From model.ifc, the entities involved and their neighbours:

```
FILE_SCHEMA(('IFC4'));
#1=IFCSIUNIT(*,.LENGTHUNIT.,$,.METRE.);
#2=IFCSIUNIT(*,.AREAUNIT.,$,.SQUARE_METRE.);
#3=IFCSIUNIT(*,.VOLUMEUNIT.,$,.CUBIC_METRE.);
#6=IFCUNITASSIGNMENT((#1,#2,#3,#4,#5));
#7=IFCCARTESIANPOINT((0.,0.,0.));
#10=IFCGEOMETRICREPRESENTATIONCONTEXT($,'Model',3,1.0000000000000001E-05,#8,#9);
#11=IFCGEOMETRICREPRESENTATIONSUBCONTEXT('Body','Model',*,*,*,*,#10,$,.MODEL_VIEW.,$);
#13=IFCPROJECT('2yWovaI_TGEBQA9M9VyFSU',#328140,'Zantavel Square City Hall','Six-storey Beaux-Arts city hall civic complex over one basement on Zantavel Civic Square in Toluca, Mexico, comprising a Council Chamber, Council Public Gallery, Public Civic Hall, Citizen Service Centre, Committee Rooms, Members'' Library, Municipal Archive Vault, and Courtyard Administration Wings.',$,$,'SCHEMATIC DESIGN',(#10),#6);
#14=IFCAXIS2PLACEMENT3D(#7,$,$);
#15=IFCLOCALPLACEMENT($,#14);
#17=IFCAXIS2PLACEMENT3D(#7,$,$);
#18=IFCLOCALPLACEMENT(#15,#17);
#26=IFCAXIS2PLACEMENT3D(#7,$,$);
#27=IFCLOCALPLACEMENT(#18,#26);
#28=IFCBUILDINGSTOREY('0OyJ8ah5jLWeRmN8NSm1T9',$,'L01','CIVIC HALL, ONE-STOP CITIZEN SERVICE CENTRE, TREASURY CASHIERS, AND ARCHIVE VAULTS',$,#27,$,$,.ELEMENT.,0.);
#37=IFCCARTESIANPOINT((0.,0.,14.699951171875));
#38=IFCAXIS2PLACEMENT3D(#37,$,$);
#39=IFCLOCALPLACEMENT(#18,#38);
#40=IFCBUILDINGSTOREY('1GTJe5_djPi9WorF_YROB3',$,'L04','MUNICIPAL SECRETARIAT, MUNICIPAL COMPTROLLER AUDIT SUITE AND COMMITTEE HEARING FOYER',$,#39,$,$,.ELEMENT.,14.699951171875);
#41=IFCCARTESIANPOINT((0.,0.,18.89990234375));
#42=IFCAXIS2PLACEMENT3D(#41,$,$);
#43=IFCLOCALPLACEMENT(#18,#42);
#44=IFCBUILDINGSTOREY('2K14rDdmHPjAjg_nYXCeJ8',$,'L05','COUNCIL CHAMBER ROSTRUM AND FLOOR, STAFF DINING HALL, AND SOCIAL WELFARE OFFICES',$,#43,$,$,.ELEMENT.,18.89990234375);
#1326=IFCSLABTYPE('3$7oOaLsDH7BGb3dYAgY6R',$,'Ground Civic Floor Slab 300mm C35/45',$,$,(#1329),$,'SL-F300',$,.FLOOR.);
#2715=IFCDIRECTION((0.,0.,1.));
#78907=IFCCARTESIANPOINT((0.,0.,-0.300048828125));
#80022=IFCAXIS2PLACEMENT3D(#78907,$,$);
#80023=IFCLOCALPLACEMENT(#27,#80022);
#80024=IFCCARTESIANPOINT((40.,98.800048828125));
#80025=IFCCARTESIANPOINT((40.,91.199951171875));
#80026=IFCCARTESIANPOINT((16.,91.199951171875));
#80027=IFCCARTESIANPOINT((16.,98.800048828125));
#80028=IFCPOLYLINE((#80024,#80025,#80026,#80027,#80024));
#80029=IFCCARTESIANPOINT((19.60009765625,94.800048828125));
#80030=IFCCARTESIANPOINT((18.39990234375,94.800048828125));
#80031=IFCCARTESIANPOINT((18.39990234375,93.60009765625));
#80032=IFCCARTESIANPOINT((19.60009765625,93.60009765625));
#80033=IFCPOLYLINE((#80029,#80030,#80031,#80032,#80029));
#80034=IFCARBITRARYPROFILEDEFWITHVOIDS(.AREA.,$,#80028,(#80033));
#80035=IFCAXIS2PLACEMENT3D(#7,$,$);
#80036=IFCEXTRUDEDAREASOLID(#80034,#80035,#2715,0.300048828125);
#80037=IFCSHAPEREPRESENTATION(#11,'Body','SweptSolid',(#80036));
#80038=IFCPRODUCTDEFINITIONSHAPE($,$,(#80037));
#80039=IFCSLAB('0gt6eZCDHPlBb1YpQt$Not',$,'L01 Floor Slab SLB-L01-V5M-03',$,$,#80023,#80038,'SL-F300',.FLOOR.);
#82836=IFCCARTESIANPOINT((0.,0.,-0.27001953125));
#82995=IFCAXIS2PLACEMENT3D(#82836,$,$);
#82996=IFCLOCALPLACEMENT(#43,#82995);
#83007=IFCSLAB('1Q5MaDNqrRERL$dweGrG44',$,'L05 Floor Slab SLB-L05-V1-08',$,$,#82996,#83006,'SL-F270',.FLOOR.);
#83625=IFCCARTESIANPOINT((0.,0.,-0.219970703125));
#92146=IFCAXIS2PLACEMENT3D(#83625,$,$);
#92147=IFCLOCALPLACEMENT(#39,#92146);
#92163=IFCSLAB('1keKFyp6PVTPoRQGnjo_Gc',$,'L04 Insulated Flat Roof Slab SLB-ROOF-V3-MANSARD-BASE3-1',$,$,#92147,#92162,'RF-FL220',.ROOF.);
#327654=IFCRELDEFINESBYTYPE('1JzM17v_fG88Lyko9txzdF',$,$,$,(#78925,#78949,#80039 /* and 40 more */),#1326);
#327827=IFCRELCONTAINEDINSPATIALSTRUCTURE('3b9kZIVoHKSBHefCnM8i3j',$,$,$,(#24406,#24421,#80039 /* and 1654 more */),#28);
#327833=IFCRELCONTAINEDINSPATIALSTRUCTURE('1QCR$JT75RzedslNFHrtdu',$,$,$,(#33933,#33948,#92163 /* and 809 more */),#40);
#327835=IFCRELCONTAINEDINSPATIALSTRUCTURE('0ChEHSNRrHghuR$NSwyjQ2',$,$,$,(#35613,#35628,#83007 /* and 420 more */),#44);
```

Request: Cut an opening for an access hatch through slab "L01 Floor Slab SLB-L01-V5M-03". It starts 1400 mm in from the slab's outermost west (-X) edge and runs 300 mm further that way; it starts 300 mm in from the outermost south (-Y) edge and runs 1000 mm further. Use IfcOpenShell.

```python
import numpy as np
import ifcopenshell
import ifcopenshell.api.feature
import ifcopenshell.api.geometry
import ifcopenshell.api.root
import ifcopenshell.geom
import ifcopenshell.util.placement
import ifcopenshell.util.representation
import ifcopenshell.util.shape
import ifcopenshell.util.unit

model = ifcopenshell.open("model.ifc")
unit_scale = ifcopenshell.util.unit.calculate_unit_scale(model)
settings = ifcopenshell.geom.settings()


def volume(element):
    """Net volume in cubic metres, openings subtracted."""
    shape = ifcopenshell.geom.create_shape(settings, element)
    return ifcopenshell.util.shape.get_volume(shape.geometry)


slab = model.by_guid("0gt6eZCDHPlBb1YpQt$Not")
before = volume(slab)

# Extent in the slab's own axes, in metres. The edges named are its -X and -Y sides.
slab_shape = ifcopenshell.geom.create_shape(settings, slab)
vertices = ifcopenshell.util.shape.get_vertices(slab_shape.geometry)
x_min, y_min, bottom = vertices.min(axis=0)
top = vertices[:, 2].max()

opening = ifcopenshell.api.root.create_entity(model, ifc_class="IfcOpeningElement", name="Access hatch opening", predefined_type="OPENING")
context = ifcopenshell.util.representation.get_context(model, "Model", "Body", "MODEL_VIEW")
width, depth = 0.3, 1
outline = [(0.0, 0.0), (width, 0.0), (width, depth), (0.0, depth), (0.0, 0.0)]
# Overshoot both faces by 50 mm so the cut is clean.
shape = ifcopenshell.api.geometry.add_slab_representation(
    model, context=context, depth=top - bottom + 0.1, polyline=outline
)
ifcopenshell.api.geometry.assign_representation(model, product=opening, representation=shape)

matrix = ifcopenshell.util.placement.get_local_placement(slab.ObjectPlacement)
matrix[:, 3] = matrix @ np.append(np.array([x_min + 1.4, y_min + 0.3, bottom - 0.05]) / unit_scale, 1.0)
ifcopenshell.api.geometry.edit_object_placement(model, product=opening, matrix=matrix, is_si=False)
ifcopenshell.api.feature.add_feature(model, feature=opening, element=slab)

after = volume(slab)

print(f"slab volume {before:.3f} -> {after:.3f} m3")

model.write("model-out.ifc")
```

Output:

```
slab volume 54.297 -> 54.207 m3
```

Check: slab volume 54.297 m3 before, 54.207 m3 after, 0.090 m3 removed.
